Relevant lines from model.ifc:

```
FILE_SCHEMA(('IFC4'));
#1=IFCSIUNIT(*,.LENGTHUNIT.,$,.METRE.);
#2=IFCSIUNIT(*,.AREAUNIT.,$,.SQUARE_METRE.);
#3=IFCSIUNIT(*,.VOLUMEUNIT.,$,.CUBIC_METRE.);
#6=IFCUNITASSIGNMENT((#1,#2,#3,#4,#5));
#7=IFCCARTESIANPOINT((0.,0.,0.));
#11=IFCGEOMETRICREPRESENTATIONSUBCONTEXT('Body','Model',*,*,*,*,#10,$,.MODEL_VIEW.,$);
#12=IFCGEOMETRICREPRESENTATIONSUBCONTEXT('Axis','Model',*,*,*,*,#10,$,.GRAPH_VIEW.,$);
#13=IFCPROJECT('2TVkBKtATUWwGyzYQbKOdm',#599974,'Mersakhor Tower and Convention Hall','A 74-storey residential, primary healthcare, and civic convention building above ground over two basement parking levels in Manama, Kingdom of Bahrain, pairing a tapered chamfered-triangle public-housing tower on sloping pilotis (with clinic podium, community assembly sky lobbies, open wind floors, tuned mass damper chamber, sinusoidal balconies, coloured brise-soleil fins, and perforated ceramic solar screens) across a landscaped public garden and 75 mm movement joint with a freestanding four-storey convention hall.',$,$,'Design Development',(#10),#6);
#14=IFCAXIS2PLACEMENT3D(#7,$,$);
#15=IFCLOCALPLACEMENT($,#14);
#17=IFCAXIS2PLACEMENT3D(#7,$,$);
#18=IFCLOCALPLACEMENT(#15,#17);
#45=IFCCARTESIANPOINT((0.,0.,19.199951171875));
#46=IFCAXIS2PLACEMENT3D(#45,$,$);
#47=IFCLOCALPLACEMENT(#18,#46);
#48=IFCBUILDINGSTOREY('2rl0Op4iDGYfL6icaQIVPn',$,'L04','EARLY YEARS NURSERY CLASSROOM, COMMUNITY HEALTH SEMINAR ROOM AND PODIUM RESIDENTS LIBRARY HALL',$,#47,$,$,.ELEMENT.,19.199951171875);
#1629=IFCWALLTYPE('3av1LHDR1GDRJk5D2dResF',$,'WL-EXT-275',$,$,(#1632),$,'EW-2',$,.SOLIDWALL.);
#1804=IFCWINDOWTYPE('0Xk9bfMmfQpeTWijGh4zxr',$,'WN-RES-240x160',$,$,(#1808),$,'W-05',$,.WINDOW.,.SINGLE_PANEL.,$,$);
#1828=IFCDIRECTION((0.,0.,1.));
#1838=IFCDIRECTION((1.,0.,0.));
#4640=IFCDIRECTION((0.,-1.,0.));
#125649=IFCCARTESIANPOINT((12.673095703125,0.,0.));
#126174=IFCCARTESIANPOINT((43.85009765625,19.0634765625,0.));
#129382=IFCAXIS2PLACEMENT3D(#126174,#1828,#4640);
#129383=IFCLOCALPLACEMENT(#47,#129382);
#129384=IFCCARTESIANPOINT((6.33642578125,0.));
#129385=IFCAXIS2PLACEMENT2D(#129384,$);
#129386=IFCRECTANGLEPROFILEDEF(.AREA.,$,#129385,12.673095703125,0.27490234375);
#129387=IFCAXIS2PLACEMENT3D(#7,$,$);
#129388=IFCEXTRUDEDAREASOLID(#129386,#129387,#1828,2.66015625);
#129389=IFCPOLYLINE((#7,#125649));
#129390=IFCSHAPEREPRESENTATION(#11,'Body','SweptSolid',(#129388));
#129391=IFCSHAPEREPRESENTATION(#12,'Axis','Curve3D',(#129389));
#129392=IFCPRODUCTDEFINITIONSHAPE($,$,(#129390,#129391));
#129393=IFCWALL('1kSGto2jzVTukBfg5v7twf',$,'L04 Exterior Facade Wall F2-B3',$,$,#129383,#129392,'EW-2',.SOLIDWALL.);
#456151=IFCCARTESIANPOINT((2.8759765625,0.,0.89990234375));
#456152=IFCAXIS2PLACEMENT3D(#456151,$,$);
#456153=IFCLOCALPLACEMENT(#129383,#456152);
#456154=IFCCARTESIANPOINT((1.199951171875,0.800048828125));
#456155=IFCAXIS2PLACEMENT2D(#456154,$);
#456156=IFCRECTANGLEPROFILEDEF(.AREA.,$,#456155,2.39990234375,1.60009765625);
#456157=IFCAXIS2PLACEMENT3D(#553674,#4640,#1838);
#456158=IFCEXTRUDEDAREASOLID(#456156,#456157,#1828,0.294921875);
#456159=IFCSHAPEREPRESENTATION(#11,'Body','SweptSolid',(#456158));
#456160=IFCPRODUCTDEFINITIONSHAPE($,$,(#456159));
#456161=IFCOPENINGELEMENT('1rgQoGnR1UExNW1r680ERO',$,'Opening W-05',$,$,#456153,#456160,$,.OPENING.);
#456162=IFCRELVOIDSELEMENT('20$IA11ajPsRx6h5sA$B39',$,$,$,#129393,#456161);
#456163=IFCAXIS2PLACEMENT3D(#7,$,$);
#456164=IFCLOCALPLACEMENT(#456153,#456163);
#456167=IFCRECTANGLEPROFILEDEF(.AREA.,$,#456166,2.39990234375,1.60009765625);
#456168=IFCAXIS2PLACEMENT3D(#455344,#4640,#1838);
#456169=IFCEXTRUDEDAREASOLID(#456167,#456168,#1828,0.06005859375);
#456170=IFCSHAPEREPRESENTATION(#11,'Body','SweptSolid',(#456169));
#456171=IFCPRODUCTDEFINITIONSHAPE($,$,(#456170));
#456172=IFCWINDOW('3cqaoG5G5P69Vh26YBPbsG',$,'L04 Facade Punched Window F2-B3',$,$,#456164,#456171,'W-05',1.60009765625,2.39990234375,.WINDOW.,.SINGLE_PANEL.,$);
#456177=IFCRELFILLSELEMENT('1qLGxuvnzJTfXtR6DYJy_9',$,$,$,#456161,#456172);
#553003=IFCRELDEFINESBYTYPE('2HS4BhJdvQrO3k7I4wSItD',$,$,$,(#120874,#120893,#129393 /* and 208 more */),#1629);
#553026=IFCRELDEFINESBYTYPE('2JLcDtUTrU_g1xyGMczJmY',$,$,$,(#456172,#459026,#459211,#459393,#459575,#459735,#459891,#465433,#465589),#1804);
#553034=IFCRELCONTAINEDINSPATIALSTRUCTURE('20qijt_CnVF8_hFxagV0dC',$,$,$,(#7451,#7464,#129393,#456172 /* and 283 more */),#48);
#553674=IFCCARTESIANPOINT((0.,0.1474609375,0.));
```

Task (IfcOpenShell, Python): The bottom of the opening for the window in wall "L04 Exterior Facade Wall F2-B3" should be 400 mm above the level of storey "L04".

```python
import numpy as np
import ifcopenshell
import ifcopenshell.api.geometry
import ifcopenshell.geom
import ifcopenshell.util.element
import ifcopenshell.util.placement
import ifcopenshell.util.shape
import ifcopenshell.util.unit

model = ifcopenshell.open("model.ifc")
unit_scale = ifcopenshell.util.unit.calculate_unit_scale(model)

window = model.by_guid("3cqaoG5G5P69Vh26YBPbsG")
opening = window.FillsVoids[0].RelatingOpeningElement
storey = ifcopenshell.util.element.get_container(window, ifc_class="IfcBuildingStorey")
level = ifcopenshell.util.placement.get_local_placement(storey.ObjectPlacement)[2, 3]

# The opening's origin need not be at the sill, so measure its lowest point.
shape = ifcopenshell.geom.create_shape(ifcopenshell.geom.settings(), opening)
bottom = ifcopenshell.util.shape.get_shape_bottom_elevation(shape, shape.geometry) / unit_scale
dz = level + 0.4 / unit_scale - bottom

shift = np.array([0.0, 0.0, dz])
# The window is placed relative to its opening, so it follows when the opening moves.
matrix = ifcopenshell.util.placement.get_local_placement(opening.ObjectPlacement)
matrix[:3, 3] += shift
ifcopenshell.api.geometry.edit_object_placement(
    model, product=opening, matrix=matrix, is_si=False, should_transform_children=True
)

print(f"moved by {dz * unit_scale:+.3f} m")

model.write("model-out.ifc")
```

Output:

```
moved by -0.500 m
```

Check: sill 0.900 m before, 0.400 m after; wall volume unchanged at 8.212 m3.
